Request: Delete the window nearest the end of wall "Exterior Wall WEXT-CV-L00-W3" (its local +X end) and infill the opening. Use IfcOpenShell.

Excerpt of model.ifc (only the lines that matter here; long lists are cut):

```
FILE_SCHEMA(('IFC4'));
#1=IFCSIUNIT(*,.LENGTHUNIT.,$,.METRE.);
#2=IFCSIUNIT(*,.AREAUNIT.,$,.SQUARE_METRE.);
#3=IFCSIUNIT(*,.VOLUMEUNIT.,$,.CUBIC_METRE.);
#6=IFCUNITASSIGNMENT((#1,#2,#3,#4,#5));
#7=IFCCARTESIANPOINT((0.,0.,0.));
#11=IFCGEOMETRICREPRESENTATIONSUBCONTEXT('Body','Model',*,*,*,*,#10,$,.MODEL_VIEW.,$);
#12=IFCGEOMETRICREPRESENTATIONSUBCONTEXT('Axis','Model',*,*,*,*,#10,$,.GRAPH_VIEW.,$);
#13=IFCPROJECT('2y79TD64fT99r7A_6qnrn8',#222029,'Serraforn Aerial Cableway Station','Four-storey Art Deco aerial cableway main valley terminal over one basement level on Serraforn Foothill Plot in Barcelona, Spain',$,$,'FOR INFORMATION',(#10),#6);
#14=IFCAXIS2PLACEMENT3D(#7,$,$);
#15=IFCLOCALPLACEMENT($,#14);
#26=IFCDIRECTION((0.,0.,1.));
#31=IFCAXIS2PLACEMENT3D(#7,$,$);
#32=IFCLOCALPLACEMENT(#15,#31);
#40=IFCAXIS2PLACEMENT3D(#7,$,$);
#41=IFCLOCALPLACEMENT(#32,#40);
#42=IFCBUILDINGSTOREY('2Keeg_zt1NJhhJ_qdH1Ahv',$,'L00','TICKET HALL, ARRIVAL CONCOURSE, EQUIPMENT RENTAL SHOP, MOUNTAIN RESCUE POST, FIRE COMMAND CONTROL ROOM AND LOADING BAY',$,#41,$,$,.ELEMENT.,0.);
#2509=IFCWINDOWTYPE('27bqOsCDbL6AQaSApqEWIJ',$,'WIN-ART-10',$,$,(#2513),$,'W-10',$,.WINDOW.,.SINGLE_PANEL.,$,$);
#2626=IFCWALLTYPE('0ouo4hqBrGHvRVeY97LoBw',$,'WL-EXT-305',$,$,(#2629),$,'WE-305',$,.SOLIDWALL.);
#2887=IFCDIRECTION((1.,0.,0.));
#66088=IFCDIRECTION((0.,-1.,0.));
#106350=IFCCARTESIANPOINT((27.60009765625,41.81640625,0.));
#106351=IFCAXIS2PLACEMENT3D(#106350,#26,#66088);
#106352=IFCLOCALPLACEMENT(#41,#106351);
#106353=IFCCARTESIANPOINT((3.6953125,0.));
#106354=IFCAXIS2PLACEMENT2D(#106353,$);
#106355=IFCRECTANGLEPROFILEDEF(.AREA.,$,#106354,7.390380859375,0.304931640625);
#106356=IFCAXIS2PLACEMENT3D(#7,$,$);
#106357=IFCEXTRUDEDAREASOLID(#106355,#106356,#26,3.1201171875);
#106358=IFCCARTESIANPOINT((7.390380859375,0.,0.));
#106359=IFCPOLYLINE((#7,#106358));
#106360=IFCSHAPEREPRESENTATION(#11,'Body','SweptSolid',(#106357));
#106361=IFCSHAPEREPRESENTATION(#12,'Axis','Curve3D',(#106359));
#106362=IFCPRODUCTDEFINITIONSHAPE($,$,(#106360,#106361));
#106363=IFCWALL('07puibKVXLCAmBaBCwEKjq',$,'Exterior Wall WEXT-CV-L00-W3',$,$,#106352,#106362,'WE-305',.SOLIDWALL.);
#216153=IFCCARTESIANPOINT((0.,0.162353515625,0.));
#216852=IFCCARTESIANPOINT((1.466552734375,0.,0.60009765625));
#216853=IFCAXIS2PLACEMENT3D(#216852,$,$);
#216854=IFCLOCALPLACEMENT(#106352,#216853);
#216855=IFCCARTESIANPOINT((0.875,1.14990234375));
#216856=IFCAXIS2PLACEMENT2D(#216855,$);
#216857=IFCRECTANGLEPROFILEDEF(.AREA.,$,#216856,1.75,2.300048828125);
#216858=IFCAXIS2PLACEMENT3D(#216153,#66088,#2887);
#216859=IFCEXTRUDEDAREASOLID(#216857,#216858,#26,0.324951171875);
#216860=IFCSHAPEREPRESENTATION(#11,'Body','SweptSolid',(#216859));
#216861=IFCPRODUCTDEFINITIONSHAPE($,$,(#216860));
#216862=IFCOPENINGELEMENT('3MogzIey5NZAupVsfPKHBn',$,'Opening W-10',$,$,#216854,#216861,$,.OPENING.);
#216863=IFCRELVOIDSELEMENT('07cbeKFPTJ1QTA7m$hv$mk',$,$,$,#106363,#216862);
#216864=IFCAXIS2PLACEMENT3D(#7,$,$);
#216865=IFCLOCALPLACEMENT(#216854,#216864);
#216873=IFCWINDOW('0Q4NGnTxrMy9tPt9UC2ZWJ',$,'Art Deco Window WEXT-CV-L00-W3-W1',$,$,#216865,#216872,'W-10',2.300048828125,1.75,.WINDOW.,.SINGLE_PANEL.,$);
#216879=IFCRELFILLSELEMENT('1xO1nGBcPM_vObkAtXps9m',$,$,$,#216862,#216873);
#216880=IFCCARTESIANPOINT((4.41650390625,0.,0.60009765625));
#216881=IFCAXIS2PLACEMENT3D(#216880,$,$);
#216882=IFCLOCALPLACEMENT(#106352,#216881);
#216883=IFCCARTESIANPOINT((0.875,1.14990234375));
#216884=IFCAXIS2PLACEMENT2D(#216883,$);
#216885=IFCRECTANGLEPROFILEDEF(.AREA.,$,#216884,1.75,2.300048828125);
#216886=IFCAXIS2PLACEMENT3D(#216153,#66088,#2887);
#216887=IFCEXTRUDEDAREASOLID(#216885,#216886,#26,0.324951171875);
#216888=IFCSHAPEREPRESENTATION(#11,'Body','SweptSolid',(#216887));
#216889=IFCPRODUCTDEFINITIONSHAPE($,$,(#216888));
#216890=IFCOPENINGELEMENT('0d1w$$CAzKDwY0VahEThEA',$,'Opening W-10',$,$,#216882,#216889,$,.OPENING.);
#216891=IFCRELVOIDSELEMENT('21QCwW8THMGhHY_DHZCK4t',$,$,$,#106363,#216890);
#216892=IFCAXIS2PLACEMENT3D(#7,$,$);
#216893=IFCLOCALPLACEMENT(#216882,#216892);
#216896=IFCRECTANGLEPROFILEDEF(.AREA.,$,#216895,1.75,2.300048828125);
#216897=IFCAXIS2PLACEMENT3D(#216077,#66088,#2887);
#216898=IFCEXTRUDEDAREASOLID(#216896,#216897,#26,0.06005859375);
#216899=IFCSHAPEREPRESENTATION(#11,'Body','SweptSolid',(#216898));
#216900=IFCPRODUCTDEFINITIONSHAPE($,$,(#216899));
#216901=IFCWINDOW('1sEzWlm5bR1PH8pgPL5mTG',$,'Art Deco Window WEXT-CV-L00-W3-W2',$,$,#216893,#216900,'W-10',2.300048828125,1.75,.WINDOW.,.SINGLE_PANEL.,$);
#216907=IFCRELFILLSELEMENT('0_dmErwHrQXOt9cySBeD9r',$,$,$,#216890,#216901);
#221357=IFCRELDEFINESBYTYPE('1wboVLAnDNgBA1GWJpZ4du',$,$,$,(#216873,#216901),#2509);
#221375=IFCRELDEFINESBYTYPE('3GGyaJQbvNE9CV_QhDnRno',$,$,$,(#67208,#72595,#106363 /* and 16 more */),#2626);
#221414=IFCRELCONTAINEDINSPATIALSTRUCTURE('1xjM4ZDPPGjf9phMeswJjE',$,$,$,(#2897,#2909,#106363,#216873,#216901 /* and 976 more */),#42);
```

```python
import ifcopenshell
import ifcopenshell.api.feature
import ifcopenshell.api.root
import ifcopenshell.geom
import ifcopenshell.util.shape

model = ifcopenshell.open("model.ifc")
settings = ifcopenshell.geom.settings()


def volume(element):
    """Net volume in cubic metres, openings subtracted."""
    shape = ifcopenshell.geom.create_shape(settings, element)
    return ifcopenshell.util.shape.get_volume(shape.geometry)


window = model.by_guid("1sEzWlm5bR1PH8pgPL5mTG")
opening = window.FillsVoids[0].RelatingOpeningElement
wall = opening.VoidsElements[0].RelatingBuildingElement
before = volume(wall)

ifcopenshell.api.root.remove_product(model, product=window)
ifcopenshell.api.feature.remove_feature(model, feature=opening)

after = volume(wall)

print(f"wall volume {before:.3f} -> {after:.3f} m3")

model.write("model_edited.ifc")
```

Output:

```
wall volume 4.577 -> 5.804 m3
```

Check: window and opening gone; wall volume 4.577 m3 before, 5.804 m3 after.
